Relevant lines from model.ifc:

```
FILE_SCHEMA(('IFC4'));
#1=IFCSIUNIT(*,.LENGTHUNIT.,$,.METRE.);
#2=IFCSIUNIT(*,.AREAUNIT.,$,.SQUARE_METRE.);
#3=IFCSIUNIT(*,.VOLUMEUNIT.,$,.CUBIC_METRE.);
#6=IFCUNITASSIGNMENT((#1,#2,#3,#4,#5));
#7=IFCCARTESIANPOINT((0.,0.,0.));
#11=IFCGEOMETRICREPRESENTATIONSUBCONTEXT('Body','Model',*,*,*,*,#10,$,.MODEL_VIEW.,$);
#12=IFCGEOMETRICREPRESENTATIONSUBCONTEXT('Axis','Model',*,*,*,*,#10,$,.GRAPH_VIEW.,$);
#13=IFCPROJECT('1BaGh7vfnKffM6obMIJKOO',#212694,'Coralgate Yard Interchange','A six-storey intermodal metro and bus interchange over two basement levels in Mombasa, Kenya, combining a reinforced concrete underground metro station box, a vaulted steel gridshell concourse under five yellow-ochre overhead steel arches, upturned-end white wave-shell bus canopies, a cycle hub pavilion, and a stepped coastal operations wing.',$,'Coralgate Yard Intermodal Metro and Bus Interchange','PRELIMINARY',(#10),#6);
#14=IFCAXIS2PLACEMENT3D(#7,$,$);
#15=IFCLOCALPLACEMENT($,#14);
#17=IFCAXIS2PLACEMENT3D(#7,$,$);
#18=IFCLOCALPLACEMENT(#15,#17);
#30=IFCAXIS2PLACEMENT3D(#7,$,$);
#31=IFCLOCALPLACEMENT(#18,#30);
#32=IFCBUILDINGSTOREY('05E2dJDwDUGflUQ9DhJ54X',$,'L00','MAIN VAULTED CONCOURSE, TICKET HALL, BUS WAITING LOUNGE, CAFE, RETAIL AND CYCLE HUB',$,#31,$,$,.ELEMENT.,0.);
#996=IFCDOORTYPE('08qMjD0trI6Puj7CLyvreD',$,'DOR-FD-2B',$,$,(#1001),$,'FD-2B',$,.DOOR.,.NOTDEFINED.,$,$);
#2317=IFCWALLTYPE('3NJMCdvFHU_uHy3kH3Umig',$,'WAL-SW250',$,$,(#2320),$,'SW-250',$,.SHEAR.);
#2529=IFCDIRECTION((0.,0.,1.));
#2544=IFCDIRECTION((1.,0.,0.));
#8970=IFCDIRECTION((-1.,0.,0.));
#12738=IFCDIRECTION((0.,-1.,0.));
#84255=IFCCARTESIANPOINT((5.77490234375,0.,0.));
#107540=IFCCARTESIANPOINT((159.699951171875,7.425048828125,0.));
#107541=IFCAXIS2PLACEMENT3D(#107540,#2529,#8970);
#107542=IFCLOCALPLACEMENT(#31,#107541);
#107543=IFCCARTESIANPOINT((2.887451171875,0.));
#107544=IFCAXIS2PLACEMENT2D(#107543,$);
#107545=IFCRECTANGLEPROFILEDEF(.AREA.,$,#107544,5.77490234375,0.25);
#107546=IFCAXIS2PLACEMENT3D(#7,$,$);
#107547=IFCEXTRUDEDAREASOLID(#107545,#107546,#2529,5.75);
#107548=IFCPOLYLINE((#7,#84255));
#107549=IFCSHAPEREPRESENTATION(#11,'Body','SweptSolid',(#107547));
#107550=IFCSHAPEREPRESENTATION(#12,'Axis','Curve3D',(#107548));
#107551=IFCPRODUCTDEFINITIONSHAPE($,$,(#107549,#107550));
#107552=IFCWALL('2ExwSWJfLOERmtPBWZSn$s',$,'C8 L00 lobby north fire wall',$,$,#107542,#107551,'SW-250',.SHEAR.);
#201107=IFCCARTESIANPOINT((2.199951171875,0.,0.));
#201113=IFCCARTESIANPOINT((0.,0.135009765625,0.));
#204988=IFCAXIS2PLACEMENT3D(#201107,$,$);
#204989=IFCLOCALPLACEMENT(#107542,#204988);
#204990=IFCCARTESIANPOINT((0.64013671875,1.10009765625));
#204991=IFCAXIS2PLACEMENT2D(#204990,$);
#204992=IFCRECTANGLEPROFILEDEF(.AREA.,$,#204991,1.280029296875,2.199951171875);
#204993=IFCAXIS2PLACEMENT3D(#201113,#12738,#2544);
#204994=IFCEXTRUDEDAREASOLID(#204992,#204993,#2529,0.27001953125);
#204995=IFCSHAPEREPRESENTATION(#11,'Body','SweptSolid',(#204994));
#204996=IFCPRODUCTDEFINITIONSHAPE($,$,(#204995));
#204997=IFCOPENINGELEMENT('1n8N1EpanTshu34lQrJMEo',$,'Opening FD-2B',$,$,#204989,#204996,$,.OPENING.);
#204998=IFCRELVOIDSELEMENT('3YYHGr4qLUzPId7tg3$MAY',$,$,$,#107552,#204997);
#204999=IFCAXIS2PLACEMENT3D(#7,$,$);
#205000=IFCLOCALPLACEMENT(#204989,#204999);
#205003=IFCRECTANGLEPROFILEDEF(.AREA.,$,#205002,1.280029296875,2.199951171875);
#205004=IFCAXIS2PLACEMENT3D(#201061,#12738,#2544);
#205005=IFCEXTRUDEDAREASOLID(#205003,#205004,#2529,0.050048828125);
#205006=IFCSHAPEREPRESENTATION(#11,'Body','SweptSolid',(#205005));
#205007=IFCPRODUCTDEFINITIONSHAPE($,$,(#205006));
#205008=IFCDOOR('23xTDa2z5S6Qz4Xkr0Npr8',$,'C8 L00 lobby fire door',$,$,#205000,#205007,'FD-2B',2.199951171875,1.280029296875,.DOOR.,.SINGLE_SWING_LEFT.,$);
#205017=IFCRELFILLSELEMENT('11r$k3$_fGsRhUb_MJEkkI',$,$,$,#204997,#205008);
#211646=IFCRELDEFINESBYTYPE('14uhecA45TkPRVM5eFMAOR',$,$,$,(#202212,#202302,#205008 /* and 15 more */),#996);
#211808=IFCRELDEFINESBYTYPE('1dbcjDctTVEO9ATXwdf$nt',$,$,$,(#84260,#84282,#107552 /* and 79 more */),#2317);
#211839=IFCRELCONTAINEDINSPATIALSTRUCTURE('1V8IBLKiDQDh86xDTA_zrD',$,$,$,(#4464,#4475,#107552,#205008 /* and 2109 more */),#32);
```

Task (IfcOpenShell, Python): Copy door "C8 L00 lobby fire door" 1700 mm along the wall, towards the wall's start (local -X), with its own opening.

```python
import ifcopenshell
import ifcopenshell.api.feature
import ifcopenshell.api.geometry
import ifcopenshell.api.root
import ifcopenshell.geom
import ifcopenshell.util.element
import ifcopenshell.util.placement
import ifcopenshell.util.shape

model = ifcopenshell.open("model.ifc")
settings = ifcopenshell.geom.settings()


def volume(element):
    """Net volume in cubic metres, openings subtracted."""
    shape = ifcopenshell.geom.create_shape(settings, element)
    return ifcopenshell.util.shape.get_volume(shape.geometry)


door = model.by_guid("23xTDa2z5S6Qz4Xkr0Npr8")
opening = door.FillsVoids[0].RelatingOpeningElement
wall = opening.VoidsElements[0].RelatingBuildingElement
before = volume(wall)
shift = ifcopenshell.util.placement.get_local_placement(wall.ObjectPlacement)[:3, 0] * -1.7

# copy_class copies the void relationship, type, container and properties, but no geometry.
new_opening = ifcopenshell.api.root.copy_class(model, product=opening)
new_opening.Representation = ifcopenshell.util.element.copy_deep(
    model, opening.Representation, exclude=["IfcGeometricRepresentationContext", "IfcRepresentationMap"]
)
new_door = ifcopenshell.api.root.copy_class(model, product=door)
new_door.Representation = ifcopenshell.util.element.copy_deep(
    model, door.Representation, exclude=["IfcGeometricRepresentationContext", "IfcRepresentationMap"]
)
new_door.Tag = None
ifcopenshell.api.feature.add_filling(model, opening=new_opening, element=new_door)

for old, new in ((opening, new_opening), (door, new_door)):
    matrix = ifcopenshell.util.placement.get_local_placement(old.ObjectPlacement)
    matrix[:3, 3] += shift
    ifcopenshell.api.geometry.edit_object_placement(model, product=new, matrix=matrix, is_si=False)

after = volume(wall)

print(f"wall volume {before:.3f} -> {after:.3f} m3")

model.write("model-out.ifc")
```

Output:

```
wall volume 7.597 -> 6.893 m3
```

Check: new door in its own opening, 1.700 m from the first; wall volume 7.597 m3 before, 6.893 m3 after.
